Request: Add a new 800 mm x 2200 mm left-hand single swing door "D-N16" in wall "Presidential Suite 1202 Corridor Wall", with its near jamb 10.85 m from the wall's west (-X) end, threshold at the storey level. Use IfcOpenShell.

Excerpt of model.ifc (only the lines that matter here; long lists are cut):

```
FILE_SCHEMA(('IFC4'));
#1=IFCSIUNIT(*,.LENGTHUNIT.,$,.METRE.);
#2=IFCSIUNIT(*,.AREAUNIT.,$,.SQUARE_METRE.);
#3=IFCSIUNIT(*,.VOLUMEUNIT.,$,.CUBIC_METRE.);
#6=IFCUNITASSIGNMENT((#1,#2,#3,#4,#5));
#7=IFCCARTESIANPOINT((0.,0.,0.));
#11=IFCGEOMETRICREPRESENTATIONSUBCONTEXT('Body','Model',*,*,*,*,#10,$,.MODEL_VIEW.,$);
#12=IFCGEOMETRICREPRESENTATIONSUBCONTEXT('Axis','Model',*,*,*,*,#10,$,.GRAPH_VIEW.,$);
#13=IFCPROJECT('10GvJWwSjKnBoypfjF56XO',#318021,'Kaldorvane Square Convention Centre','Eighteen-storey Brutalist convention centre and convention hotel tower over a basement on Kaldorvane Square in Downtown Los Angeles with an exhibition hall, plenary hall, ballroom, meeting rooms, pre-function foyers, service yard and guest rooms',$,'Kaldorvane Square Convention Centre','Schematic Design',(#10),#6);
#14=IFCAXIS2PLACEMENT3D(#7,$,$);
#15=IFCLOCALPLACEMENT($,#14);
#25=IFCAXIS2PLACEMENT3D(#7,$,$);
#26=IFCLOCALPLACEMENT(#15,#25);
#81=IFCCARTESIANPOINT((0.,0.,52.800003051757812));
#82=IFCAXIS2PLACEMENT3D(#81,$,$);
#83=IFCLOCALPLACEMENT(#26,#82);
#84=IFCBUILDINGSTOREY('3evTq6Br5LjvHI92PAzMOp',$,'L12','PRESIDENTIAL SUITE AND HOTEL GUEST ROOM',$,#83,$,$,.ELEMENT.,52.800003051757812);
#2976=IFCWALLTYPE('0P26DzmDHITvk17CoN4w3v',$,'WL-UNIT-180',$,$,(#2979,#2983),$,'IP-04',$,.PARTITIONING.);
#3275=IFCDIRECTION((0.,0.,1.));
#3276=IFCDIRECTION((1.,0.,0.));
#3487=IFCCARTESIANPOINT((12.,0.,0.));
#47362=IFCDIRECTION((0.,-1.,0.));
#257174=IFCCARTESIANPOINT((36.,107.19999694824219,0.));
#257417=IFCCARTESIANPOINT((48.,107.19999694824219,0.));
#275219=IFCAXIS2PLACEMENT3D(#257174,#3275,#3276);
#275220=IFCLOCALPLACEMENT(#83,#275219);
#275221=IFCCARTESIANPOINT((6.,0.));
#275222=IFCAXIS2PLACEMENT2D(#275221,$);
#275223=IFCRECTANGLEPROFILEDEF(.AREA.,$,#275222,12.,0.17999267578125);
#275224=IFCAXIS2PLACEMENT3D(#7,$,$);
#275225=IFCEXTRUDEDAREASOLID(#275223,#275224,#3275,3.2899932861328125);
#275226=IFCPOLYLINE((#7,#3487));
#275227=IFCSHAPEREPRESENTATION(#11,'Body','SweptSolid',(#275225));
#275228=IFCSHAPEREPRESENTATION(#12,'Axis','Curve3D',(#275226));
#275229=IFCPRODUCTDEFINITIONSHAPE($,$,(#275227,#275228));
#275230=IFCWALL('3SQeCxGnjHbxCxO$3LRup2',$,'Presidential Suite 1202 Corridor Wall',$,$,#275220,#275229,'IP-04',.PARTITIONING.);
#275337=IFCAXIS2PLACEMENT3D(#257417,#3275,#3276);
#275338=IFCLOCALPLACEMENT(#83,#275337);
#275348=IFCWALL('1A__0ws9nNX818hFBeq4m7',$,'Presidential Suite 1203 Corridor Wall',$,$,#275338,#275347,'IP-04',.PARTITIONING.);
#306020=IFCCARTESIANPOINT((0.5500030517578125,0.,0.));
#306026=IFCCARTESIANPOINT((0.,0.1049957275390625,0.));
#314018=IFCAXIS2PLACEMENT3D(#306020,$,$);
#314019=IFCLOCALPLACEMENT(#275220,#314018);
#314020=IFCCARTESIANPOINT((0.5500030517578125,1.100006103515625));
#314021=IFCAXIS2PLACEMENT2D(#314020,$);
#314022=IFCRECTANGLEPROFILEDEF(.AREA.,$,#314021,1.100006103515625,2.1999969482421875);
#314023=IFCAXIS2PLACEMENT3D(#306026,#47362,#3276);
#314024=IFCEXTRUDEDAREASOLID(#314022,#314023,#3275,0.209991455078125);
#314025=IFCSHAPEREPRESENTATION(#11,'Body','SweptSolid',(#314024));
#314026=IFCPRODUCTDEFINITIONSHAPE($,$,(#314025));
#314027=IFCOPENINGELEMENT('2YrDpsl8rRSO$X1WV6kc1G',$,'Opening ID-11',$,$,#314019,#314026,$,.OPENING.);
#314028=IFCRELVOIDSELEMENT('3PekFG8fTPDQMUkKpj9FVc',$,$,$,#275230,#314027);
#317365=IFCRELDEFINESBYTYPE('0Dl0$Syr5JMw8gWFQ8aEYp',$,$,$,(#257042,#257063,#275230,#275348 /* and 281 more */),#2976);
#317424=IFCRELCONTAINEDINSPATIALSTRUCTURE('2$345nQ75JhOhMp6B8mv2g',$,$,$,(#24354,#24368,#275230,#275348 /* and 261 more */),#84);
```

```python
import numpy as np
import ifcopenshell
import ifcopenshell.api.feature
import ifcopenshell.api.geometry
import ifcopenshell.api.root
import ifcopenshell.api.spatial
import ifcopenshell.geom
import ifcopenshell.util.element
import ifcopenshell.util.placement
import ifcopenshell.util.representation
import ifcopenshell.util.shape
import ifcopenshell.util.unit

model = ifcopenshell.open("model.ifc")
unit_scale = ifcopenshell.util.unit.calculate_unit_scale(model)
settings = ifcopenshell.geom.settings()


def volume(element):
    """Net volume in cubic metres, openings subtracted."""
    shape = ifcopenshell.geom.create_shape(settings, element)
    return ifcopenshell.util.shape.get_volume(shape.geometry)


wall = model.by_guid("3SQeCxGnjHbxCxO$3LRup2")
storey = ifcopenshell.util.element.get_container(wall, ifc_class="IfcBuildingStorey")
context = ifcopenshell.util.representation.get_context(model, "Model", "Body", "MODEL_VIEW")
before = volume(wall)

width, height, from_end, sill = 0.8, 2.2, 10.85, 0.0  # metres

# The wall runs along its own X axis, and the end named is its -X end.
wall_shape = ifcopenshell.geom.create_shape(settings, wall)
x, y, z = ifcopenshell.util.shape.get_vertices(wall_shape.geometry).T
start = x.min() + from_end
face, thickness = float(y.min()), float(y.max() - y.min())
wall_matrix = ifcopenshell.util.placement.get_local_placement(wall.ObjectPlacement)
level = ifcopenshell.util.placement.get_local_placement(storey.ObjectPlacement)[2, 3]


def in_wall(x, y):
    """Placement at x, y metres in the wall's axes, at sill height."""
    matrix = wall_matrix.copy()
    matrix[:, 3] = wall_matrix @ np.array([x / unit_scale, y / unit_scale, 0.0, 1.0])
    matrix[2, 3] = level + sill / unit_scale
    return matrix


# Opening: a box that overshoots both wall faces by 50 mm.
opening = ifcopenshell.api.root.create_entity(model, ifc_class="IfcOpeningElement", predefined_type="OPENING")
box = ifcopenshell.api.geometry.add_wall_representation(
    model, context=context, length=width, height=height, thickness=thickness + 0.1
)
ifcopenshell.api.geometry.assign_representation(model, product=opening, representation=box)
ifcopenshell.api.geometry.edit_object_placement(model, product=opening, matrix=in_wall(start, face - 0.05), is_si=False)
ifcopenshell.api.feature.add_feature(model, feature=opening, element=wall)

door = ifcopenshell.api.root.create_entity(model, ifc_class="IfcDoor", name="D-N16", predefined_type="DOOR")
door.OverallWidth, door.OverallHeight = width / unit_scale, height / unit_scale
door.OperationType = "SINGLE_SWING_LEFT"
body = ifcopenshell.api.geometry.add_door_representation(
    model,
    context=context,
    overall_width=door.OverallWidth,
    overall_height=door.OverallHeight,
    operation_type="SINGLE_SWING_LEFT",
    lining_properties={"LiningDepth": thickness / unit_scale, "ThresholdDepth": thickness / unit_scale},
)
ifcopenshell.api.geometry.assign_representation(model, product=door, representation=body)
ifcopenshell.api.spatial.assign_container(model, products=[door], relating_structure=storey)
ifcopenshell.api.feature.add_filling(model, opening=opening, element=door)

# The lining spans the wall, so the door starts at the wall face.
ifcopenshell.api.geometry.edit_object_placement(model, product=door, matrix=in_wall(start, face), is_si=False)

after = volume(wall)

print(f"wall volume {before:.3f} -> {after:.3f} m3")

model.write("model_updated.ifc")
```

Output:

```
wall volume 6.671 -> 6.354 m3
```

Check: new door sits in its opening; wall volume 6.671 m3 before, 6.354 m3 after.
